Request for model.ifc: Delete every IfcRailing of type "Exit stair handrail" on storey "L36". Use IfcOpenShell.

First a look at what the model holds.

```python
import ifcopenshell
import ifcopenshell.util.element

model = ifcopenshell.open("model.ifc")
print(model.schema)
storey = next(s for s in model.by_type("IfcBuildingStorey") if s.Name == "L36")
railings = [e for e in ifcopenshell.util.element.get_decomposition(storey) if e.is_a("IfcRailing")]
seen = {}
for e in railings:
    element_type = ifcopenshell.util.element.get_type(e)
    name = element_type.Name if element_type not in (None, e) else None
    seen[name] = seen.get(name, 0) + 1
for name, count in sorted(seen.items(), key=str):
    print(count, "x", name)
```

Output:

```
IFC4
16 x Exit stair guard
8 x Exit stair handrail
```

```python
import ifcopenshell
import ifcopenshell.api.root
import ifcopenshell.util.element

model = ifcopenshell.open("model.ifc")

storey = next(s for s in model.by_type("IfcBuildingStorey") if s.Name == "L36")
railings = [e for e in ifcopenshell.util.element.get_decomposition(storey) if e.is_a("IfcRailing")]
targets = [e for e in railings if (t := ifcopenshell.util.element.get_type(e)) not in (None, e) and t.Name == "Exit stair handrail"]

for e in targets:
    ifcopenshell.api.root.remove_product(model, product=e)
print(len(targets), "removed")

model.write("model-out.ifc")
```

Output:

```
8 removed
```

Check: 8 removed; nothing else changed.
